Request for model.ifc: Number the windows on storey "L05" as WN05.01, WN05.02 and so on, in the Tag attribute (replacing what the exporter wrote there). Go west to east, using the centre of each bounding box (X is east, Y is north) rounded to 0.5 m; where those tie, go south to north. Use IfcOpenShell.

First a look at what the model holds.

```python
import ifcopenshell
import ifcopenshell.util.element
import ifcopenshell.util.placement

model = ifcopenshell.open("model.ifc")
print(model.schema)
storey = next(s for s in model.by_type("IfcBuildingStorey") if s.Name == "L05")
windows = [e for e in ifcopenshell.util.element.get_decomposition(storey) if e.is_a("IfcWindow")]
for e in sorted(windows, key=lambda e: e.id()):
    origin = ifcopenshell.util.placement.get_local_placement(e.ObjectPlacement)[:3, 3]
    print(e.id(), e.Tag, e.Name, origin.round(2) + 0.0, sep=" | ")
```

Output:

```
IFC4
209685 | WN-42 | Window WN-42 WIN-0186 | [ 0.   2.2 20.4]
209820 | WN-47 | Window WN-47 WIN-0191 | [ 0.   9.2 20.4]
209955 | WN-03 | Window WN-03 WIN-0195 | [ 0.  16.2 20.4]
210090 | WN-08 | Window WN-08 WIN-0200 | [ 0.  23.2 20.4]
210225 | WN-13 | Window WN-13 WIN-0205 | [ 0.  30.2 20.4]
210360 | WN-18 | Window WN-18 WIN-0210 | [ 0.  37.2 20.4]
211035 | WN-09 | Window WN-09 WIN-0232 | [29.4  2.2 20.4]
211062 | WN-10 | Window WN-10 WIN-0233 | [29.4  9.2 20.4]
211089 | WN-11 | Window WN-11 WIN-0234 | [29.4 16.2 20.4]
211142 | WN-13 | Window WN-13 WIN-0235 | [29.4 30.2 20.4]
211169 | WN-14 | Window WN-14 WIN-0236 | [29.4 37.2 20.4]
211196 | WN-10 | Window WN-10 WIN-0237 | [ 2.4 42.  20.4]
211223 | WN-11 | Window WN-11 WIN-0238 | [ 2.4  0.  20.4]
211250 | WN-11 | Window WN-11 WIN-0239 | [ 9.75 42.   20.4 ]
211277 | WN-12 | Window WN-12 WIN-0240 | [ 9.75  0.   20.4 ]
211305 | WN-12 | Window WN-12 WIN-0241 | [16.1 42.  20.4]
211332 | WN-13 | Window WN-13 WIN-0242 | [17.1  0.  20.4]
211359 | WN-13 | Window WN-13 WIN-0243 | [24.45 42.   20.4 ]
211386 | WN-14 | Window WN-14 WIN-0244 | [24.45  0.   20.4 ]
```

```python
import ifcopenshell
import ifcopenshell.geom
import ifcopenshell.util.element
import ifcopenshell.util.shape

model = ifcopenshell.open("model.ifc")
settings = ifcopenshell.geom.settings()
settings.set("use-world-coords", True)


def centre(element):
    shape = ifcopenshell.geom.create_shape(settings, element)
    return ifcopenshell.util.shape.get_bbox_centroid(shape.geometry)


storey = next(s for s in model.by_type("IfcBuildingStorey") if s.Name == "L05")
windows = [e for e in ifcopenshell.util.element.get_decomposition(storey) if e.is_a("IfcWindow")]

# Insertion points can sit at a corner or the storey origin, so sort by the geometry (in metres).
centres = {e: centre(e) for e in windows}
windows.sort(key=lambda e: (round(centres[e][0] / 0.5), centres[e][1]))

for i, e in enumerate(windows, start=1):
    number = f"WN05.{i:02d}"
    e.Tag = number
    print(e.id(), number)

model.write("model_edited.ifc")
```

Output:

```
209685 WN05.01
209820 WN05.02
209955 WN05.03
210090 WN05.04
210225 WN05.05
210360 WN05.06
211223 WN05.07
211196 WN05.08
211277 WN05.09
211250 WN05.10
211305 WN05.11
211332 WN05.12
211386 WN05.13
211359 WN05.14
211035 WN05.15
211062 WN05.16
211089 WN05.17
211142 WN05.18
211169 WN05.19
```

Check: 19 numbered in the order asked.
